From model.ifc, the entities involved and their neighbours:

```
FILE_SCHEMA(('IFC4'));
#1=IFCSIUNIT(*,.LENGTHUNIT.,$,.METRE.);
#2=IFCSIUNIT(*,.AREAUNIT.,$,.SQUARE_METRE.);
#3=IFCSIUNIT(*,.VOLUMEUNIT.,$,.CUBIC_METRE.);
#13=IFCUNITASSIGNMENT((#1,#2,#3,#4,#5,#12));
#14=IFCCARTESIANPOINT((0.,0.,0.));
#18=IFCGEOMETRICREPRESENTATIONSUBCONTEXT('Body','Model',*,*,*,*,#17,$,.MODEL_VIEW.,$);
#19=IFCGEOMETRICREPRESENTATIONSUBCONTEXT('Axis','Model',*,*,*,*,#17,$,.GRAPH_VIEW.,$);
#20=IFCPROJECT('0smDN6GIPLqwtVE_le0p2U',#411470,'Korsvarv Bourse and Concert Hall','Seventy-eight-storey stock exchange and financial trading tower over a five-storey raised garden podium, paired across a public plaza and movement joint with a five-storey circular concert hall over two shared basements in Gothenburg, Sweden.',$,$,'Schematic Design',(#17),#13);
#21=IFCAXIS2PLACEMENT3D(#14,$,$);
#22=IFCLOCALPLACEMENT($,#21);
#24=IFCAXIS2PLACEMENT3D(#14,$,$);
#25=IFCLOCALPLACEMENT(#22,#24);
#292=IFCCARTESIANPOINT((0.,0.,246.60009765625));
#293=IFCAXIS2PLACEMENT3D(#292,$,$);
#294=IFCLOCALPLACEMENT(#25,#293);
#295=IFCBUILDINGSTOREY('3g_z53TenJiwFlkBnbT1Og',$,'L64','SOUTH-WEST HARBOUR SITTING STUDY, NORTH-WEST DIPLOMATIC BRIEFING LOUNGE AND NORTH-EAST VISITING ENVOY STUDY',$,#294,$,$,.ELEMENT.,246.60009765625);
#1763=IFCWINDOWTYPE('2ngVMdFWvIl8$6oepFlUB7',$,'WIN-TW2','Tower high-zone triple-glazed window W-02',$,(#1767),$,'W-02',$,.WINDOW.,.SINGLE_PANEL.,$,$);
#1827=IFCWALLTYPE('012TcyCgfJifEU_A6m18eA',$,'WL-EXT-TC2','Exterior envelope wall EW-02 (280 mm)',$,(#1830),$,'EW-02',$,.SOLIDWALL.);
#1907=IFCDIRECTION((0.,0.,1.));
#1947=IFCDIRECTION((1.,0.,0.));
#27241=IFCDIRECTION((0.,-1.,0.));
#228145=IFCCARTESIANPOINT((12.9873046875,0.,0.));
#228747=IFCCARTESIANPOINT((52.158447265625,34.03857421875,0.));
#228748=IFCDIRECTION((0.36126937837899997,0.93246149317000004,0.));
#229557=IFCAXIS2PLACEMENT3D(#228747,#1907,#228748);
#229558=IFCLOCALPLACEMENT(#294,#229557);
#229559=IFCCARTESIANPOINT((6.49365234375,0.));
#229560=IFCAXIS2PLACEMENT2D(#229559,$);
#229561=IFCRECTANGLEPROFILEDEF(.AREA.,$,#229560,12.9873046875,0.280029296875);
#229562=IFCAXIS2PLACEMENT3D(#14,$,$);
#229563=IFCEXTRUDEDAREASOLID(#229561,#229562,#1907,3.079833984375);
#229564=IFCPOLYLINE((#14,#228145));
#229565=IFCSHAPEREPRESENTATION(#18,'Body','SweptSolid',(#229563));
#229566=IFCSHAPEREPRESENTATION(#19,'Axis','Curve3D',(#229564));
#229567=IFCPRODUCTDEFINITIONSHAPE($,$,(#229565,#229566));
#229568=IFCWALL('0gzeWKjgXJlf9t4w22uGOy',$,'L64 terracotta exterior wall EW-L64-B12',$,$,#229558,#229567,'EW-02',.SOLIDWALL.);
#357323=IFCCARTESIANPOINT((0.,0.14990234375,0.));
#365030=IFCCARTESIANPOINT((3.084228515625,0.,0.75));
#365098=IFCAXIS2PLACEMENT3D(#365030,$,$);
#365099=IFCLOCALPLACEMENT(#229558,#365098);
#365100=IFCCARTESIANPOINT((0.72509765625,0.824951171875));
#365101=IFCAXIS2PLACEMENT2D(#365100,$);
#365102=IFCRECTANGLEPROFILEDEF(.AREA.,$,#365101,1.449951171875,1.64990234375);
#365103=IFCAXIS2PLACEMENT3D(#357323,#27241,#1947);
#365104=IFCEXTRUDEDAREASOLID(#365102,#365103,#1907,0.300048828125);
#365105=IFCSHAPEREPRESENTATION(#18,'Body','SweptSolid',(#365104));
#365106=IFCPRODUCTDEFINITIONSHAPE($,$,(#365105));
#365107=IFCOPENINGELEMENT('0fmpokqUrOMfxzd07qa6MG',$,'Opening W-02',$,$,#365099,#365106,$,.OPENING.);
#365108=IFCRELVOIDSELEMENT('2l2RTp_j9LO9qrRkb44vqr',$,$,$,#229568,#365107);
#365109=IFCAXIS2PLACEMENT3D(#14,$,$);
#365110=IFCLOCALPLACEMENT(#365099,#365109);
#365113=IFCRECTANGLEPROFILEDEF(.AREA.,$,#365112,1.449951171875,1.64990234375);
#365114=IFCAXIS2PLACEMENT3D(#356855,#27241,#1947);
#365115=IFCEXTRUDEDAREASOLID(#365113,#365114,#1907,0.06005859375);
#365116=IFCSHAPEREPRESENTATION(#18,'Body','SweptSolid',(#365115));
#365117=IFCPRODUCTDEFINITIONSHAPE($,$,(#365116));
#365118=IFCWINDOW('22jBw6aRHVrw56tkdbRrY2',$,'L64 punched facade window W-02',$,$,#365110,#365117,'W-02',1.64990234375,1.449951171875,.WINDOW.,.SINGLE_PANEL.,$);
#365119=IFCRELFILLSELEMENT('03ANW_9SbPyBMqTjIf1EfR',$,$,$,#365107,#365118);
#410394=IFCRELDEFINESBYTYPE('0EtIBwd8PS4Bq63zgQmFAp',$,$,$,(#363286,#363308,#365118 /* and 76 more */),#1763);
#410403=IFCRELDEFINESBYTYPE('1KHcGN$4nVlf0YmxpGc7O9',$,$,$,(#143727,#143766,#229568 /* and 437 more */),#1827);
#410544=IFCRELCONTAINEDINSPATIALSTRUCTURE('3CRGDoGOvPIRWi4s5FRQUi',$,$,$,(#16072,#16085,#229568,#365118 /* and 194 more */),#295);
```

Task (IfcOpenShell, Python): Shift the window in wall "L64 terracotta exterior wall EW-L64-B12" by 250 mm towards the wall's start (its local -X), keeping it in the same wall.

```python
import ifcopenshell
import ifcopenshell.api.geometry
import ifcopenshell.util.placement
import ifcopenshell.util.unit

model = ifcopenshell.open("model.ifc")
unit_scale = ifcopenshell.util.unit.calculate_unit_scale(model)

window = model.by_guid("22jBw6aRHVrw56tkdbRrY2")
opening = window.FillsVoids[0].RelatingOpeningElement
wall = opening.VoidsElements[0].RelatingBuildingElement

wall_matrix = ifcopenshell.util.placement.get_local_placement(wall.ObjectPlacement)
shift = wall_matrix[:3, 0] * -0.25 / unit_scale
before = ifcopenshell.util.placement.get_local_placement(window.ObjectPlacement)[:3, 3].copy()

# The window is placed relative to its opening, so it follows when the opening moves.
matrix = ifcopenshell.util.placement.get_local_placement(opening.ObjectPlacement)
matrix[:3, 3] += shift
ifcopenshell.api.geometry.edit_object_placement(
    model, product=opening, matrix=matrix, is_si=False, should_transform_children=True
)

after = ifcopenshell.util.placement.get_local_placement(window.ObjectPlacement)[:3, 3]
print("window moved by", (after - before).round(3) + 0.0)

model.write("model_v2.ifc")
```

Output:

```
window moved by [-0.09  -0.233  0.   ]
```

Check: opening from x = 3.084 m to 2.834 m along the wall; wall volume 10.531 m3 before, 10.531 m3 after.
